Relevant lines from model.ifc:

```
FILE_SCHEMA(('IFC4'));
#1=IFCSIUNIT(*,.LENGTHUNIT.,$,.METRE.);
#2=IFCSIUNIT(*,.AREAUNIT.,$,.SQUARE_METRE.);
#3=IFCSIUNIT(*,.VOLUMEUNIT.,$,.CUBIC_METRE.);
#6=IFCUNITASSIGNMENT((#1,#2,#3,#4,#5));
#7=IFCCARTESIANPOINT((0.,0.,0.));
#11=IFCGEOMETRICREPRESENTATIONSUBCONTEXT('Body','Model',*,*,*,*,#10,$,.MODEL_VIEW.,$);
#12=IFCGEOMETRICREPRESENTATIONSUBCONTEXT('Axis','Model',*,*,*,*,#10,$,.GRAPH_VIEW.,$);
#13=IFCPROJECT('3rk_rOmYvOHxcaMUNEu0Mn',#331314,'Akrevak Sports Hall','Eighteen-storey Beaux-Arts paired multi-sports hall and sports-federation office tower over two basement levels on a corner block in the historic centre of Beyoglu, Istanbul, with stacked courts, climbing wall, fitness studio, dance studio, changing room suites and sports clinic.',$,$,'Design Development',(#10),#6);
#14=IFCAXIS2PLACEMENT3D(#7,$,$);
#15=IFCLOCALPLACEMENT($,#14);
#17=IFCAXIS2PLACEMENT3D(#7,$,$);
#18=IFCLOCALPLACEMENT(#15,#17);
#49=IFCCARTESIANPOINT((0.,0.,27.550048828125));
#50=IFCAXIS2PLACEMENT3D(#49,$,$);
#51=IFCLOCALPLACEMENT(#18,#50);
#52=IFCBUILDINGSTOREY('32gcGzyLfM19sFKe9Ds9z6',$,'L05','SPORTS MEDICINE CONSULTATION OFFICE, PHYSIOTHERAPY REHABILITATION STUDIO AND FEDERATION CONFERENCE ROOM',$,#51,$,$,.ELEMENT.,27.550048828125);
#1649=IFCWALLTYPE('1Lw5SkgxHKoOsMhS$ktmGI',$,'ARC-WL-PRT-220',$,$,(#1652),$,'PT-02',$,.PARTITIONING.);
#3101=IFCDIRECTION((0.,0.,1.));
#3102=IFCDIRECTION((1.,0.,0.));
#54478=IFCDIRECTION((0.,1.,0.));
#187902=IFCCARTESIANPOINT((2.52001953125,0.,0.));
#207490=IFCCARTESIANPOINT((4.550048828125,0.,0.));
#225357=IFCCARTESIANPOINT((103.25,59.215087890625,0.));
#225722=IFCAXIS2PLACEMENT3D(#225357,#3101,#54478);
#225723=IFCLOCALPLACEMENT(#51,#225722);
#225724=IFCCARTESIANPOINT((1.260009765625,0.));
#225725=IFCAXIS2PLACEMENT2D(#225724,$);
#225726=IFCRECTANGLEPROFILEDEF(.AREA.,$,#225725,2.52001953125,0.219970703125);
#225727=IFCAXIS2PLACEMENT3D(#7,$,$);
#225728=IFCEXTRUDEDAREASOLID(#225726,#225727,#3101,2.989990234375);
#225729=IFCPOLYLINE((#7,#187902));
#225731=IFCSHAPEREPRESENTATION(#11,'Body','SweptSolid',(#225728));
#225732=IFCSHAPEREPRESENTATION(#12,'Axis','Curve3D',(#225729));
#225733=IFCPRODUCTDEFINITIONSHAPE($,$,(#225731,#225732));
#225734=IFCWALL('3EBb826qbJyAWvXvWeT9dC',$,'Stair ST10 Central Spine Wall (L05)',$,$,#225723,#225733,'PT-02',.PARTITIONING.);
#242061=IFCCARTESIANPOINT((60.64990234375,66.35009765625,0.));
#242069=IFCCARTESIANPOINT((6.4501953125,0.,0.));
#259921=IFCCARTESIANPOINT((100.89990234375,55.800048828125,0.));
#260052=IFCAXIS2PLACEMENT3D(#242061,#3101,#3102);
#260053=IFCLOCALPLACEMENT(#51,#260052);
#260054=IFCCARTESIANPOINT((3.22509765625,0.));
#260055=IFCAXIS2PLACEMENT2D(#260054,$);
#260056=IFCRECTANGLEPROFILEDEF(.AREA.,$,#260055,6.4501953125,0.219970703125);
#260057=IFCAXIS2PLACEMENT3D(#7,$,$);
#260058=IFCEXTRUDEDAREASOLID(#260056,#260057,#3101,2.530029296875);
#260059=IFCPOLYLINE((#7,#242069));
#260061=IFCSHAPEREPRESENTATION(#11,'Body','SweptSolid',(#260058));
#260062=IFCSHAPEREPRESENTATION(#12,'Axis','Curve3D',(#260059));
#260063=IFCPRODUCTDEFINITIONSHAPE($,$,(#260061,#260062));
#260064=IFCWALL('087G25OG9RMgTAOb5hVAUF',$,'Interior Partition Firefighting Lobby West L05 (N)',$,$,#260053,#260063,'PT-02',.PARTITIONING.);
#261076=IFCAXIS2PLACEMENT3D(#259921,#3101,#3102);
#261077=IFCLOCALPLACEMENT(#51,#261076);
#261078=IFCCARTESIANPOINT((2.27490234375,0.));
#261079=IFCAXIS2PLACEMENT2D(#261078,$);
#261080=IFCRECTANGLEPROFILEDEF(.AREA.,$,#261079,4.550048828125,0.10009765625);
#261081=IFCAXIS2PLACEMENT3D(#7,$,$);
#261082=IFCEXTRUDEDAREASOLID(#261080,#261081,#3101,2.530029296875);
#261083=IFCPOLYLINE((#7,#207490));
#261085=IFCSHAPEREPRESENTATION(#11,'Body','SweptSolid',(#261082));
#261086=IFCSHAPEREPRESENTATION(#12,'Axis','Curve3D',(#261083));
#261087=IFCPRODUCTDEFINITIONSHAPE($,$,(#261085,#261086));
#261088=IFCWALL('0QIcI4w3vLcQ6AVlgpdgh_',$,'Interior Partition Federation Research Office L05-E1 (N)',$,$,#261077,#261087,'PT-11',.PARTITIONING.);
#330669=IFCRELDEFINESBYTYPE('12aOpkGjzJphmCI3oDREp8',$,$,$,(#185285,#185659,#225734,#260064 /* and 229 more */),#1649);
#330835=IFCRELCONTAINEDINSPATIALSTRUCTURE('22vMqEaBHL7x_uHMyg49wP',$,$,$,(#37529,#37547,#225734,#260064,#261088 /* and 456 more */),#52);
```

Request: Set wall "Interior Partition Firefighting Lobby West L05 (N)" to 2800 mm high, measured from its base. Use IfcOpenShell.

```python
import ifcopenshell
import ifcopenshell.geom
import ifcopenshell.util.representation
import ifcopenshell.util.shape

model = ifcopenshell.open("model.ifc")
settings = ifcopenshell.geom.settings()


def volume(element):
    """Net volume in cubic metres, openings subtracted."""
    shape = ifcopenshell.geom.create_shape(settings, element)
    return ifcopenshell.util.shape.get_volume(shape.geometry)


wall = model.by_guid("087G25OG9RMgTAOb5hVAUF")
before = volume(wall)

body = ifcopenshell.util.representation.get_representation(wall, "Model", "Body")
solid = body.Items[0]
old_height = solid.Depth
solid.Depth = 2.8
after = volume(wall)

print(f"height {old_height:g} -> {solid.Depth:g}, volume {before:.3f} -> {after:.3f} m3")

model.write("model_rev.ifc")
```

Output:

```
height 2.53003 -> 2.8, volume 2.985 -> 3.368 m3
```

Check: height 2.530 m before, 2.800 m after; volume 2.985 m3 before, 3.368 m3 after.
